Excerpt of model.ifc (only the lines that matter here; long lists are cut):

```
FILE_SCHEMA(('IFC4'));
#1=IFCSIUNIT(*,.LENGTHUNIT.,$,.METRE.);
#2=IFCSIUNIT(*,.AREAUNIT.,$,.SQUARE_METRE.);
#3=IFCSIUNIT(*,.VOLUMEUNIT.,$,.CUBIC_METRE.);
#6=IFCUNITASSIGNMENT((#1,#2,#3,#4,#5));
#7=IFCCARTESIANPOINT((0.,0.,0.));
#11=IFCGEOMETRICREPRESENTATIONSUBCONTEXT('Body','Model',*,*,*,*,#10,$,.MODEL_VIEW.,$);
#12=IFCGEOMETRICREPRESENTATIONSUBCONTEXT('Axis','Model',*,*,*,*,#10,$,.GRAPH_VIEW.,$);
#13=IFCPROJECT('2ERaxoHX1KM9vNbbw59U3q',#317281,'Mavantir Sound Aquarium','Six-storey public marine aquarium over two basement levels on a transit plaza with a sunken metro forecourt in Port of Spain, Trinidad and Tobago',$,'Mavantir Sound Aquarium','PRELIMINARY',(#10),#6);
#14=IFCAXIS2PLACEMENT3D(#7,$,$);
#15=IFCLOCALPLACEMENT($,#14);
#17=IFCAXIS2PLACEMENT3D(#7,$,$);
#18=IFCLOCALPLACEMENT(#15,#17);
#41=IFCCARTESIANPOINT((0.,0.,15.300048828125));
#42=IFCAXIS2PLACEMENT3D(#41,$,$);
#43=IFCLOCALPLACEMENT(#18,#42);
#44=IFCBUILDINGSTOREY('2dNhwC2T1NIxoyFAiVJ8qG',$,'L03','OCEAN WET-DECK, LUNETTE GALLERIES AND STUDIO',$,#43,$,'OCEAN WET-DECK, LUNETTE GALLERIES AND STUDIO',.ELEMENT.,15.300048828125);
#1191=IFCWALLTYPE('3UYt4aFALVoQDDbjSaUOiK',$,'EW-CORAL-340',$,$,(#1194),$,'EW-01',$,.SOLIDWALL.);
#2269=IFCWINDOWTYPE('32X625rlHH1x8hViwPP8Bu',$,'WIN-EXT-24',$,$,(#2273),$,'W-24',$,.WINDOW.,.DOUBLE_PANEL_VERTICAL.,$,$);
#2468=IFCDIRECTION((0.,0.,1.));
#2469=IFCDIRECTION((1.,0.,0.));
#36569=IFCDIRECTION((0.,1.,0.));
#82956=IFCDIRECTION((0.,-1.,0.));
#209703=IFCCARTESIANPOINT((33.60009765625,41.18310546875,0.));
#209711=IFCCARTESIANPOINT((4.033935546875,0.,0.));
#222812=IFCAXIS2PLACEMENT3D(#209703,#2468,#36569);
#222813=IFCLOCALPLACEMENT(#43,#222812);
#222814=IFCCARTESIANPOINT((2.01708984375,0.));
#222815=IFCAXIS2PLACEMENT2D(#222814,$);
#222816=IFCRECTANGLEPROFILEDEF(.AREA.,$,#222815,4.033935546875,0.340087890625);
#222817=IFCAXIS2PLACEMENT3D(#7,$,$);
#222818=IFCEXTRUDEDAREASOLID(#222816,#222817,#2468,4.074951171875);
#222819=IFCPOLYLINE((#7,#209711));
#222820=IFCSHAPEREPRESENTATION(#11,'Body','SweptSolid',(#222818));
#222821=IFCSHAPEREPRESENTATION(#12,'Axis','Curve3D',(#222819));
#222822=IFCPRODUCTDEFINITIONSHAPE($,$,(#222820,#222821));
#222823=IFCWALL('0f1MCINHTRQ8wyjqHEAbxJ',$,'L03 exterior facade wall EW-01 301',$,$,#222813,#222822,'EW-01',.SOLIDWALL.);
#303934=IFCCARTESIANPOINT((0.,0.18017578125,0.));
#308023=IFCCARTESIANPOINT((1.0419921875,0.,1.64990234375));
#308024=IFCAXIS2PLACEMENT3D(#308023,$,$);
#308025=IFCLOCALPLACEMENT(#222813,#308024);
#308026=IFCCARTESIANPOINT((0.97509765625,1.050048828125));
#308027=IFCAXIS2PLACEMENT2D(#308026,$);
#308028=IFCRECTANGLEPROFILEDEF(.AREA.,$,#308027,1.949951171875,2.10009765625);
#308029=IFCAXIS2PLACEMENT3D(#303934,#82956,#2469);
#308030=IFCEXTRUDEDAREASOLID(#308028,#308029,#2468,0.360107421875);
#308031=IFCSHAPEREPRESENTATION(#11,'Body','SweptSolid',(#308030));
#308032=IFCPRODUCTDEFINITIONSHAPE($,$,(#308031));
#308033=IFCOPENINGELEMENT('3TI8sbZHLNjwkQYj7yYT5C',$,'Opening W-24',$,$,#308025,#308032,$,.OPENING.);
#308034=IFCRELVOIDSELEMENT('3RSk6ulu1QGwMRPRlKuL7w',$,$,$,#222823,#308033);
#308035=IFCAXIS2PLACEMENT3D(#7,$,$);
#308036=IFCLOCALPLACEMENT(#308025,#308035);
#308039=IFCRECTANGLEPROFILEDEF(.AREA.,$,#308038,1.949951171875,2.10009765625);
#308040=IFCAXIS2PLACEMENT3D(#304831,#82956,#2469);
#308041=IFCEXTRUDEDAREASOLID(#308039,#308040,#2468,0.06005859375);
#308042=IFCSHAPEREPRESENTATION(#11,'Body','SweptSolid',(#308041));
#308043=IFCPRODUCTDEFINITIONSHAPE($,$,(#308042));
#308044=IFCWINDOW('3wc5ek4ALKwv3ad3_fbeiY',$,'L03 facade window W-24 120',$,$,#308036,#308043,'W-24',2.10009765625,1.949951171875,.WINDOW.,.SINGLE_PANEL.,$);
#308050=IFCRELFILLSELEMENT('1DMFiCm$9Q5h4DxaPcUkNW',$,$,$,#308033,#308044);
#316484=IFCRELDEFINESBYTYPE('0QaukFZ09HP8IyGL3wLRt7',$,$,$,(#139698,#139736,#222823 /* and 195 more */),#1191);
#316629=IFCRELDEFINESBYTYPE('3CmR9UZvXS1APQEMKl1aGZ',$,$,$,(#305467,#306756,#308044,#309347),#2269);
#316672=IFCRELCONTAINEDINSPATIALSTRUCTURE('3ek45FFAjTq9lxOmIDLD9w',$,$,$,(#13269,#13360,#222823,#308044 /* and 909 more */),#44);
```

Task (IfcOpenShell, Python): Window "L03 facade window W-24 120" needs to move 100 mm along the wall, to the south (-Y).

```python
import ifcopenshell
import ifcopenshell.api.geometry
import ifcopenshell.util.placement
import ifcopenshell.util.unit

model = ifcopenshell.open("model.ifc")
unit_scale = ifcopenshell.util.unit.calculate_unit_scale(model)

window = model.by_guid("3wc5ek4ALKwv3ad3_fbeiY")
opening = window.FillsVoids[0].RelatingOpeningElement
wall = opening.VoidsElements[0].RelatingBuildingElement

wall_matrix = ifcopenshell.util.placement.get_local_placement(wall.ObjectPlacement)
shift = wall_matrix[:3, 0] * -0.1 / unit_scale
before = ifcopenshell.util.placement.get_local_placement(window.ObjectPlacement)[:3, 3].copy()

# The window is placed relative to its opening, so it follows when the opening moves.
matrix = ifcopenshell.util.placement.get_local_placement(opening.ObjectPlacement)
matrix[:3, 3] += shift
ifcopenshell.api.geometry.edit_object_placement(
    model, product=opening, matrix=matrix, is_si=False, should_transform_children=True
)

after = ifcopenshell.util.placement.get_local_placement(window.ObjectPlacement)[:3, 3]
print("window moved by", (after - before).round(3) + 0.0)

model.write("model_edited.ifc")
```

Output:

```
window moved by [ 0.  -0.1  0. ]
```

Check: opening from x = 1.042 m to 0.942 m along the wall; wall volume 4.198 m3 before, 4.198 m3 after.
